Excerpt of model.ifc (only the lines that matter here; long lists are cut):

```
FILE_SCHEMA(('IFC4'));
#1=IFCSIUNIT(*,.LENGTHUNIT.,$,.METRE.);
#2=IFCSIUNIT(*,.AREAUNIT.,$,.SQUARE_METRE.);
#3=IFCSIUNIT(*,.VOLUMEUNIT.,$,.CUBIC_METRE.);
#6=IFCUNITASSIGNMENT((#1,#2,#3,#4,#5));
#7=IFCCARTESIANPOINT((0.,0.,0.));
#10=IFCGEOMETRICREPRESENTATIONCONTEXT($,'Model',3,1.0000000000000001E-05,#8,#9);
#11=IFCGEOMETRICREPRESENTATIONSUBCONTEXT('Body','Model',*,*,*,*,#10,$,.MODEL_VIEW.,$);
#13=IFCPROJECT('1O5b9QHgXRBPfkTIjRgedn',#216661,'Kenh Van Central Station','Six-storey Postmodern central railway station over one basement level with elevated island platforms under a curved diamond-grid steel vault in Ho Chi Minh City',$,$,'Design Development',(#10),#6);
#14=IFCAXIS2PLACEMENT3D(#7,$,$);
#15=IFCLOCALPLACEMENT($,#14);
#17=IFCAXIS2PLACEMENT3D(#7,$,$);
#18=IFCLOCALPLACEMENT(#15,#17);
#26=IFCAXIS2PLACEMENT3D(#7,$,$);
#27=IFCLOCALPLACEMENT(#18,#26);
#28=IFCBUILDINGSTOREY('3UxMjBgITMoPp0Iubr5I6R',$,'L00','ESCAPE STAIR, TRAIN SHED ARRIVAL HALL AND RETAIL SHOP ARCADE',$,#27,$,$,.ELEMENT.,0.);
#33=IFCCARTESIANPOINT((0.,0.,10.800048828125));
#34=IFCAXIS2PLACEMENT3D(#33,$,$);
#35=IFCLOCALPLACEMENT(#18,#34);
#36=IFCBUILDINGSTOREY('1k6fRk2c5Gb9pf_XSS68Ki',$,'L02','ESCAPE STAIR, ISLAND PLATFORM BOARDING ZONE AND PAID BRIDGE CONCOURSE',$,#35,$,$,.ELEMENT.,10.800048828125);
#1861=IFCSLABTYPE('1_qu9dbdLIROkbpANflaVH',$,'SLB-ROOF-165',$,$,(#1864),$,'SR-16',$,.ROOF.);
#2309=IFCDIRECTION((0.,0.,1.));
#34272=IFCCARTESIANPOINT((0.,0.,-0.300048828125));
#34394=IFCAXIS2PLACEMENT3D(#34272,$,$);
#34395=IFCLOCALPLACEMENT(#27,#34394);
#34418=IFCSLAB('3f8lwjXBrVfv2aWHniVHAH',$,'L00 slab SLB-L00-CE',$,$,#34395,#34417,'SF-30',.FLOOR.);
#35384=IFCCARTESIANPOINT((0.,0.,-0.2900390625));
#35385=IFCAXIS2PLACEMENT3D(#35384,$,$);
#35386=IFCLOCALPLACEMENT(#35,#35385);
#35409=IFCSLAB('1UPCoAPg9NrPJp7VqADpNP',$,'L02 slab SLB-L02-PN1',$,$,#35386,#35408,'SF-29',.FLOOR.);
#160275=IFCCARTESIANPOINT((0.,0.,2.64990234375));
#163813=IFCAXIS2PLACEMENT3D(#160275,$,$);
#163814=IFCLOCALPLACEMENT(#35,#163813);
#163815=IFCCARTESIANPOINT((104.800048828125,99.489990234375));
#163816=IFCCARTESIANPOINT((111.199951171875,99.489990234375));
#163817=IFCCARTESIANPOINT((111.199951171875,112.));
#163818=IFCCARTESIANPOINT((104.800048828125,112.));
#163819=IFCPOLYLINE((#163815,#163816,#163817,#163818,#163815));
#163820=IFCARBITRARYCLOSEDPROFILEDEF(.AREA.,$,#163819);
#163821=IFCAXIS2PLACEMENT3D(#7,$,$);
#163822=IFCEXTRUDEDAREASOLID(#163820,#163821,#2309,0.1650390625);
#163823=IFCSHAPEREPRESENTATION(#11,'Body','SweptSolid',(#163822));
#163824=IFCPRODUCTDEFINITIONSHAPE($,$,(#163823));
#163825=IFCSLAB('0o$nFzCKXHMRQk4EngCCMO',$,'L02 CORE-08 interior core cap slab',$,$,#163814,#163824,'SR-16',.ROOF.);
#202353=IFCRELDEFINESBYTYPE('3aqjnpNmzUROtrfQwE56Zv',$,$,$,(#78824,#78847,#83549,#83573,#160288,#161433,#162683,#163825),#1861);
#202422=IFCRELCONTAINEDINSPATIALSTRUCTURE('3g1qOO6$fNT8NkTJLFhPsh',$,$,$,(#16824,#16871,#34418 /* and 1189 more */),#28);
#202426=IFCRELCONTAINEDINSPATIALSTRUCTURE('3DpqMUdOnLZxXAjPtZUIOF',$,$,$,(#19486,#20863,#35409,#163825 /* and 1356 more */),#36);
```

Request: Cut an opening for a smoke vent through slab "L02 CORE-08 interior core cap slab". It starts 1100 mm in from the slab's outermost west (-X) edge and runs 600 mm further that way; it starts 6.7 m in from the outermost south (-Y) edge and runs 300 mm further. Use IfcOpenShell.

```python
import numpy as np
import ifcopenshell
import ifcopenshell.api.feature
import ifcopenshell.api.geometry
import ifcopenshell.api.root
import ifcopenshell.geom
import ifcopenshell.util.placement
import ifcopenshell.util.representation
import ifcopenshell.util.shape
import ifcopenshell.util.unit

model = ifcopenshell.open("model.ifc")
unit_scale = ifcopenshell.util.unit.calculate_unit_scale(model)
settings = ifcopenshell.geom.settings()


def volume(element):
    """Net volume in cubic metres, openings subtracted."""
    shape = ifcopenshell.geom.create_shape(settings, element)
    return ifcopenshell.util.shape.get_volume(shape.geometry)


slab = model.by_guid("0o$nFzCKXHMRQk4EngCCMO")
before = volume(slab)

# Extent in the slab's own axes, in metres. The edges named are its -X and -Y sides.
slab_shape = ifcopenshell.geom.create_shape(settings, slab)
vertices = ifcopenshell.util.shape.get_vertices(slab_shape.geometry)
x_min, y_min, bottom = vertices.min(axis=0)
top = vertices[:, 2].max()

opening = ifcopenshell.api.root.create_entity(model, ifc_class="IfcOpeningElement", name="Smoke vent opening", predefined_type="OPENING")
context = ifcopenshell.util.representation.get_context(model, "Model", "Body", "MODEL_VIEW")
width, depth = 0.6, 0.3
outline = [(0.0, 0.0), (width, 0.0), (width, depth), (0.0, depth), (0.0, 0.0)]
# Overshoot both faces by 50 mm so the cut is clean.
shape = ifcopenshell.api.geometry.add_slab_representation(
    model, context=context, depth=top - bottom + 0.1, polyline=outline
)
ifcopenshell.api.geometry.assign_representation(model, product=opening, representation=shape)

matrix = ifcopenshell.util.placement.get_local_placement(slab.ObjectPlacement)
matrix[:, 3] = matrix @ np.append(np.array([x_min + 1.1, y_min + 6.7, bottom - 0.05]) / unit_scale, 1.0)
ifcopenshell.api.geometry.edit_object_placement(model, product=opening, matrix=matrix, is_si=False)
ifcopenshell.api.feature.add_feature(model, feature=opening, element=slab)

after = volume(slab)

print(f"slab volume {before:.3f} -> {after:.3f} m3")

model.write("model_edited.ifc")
```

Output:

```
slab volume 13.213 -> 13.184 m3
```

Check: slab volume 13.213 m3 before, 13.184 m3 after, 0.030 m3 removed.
